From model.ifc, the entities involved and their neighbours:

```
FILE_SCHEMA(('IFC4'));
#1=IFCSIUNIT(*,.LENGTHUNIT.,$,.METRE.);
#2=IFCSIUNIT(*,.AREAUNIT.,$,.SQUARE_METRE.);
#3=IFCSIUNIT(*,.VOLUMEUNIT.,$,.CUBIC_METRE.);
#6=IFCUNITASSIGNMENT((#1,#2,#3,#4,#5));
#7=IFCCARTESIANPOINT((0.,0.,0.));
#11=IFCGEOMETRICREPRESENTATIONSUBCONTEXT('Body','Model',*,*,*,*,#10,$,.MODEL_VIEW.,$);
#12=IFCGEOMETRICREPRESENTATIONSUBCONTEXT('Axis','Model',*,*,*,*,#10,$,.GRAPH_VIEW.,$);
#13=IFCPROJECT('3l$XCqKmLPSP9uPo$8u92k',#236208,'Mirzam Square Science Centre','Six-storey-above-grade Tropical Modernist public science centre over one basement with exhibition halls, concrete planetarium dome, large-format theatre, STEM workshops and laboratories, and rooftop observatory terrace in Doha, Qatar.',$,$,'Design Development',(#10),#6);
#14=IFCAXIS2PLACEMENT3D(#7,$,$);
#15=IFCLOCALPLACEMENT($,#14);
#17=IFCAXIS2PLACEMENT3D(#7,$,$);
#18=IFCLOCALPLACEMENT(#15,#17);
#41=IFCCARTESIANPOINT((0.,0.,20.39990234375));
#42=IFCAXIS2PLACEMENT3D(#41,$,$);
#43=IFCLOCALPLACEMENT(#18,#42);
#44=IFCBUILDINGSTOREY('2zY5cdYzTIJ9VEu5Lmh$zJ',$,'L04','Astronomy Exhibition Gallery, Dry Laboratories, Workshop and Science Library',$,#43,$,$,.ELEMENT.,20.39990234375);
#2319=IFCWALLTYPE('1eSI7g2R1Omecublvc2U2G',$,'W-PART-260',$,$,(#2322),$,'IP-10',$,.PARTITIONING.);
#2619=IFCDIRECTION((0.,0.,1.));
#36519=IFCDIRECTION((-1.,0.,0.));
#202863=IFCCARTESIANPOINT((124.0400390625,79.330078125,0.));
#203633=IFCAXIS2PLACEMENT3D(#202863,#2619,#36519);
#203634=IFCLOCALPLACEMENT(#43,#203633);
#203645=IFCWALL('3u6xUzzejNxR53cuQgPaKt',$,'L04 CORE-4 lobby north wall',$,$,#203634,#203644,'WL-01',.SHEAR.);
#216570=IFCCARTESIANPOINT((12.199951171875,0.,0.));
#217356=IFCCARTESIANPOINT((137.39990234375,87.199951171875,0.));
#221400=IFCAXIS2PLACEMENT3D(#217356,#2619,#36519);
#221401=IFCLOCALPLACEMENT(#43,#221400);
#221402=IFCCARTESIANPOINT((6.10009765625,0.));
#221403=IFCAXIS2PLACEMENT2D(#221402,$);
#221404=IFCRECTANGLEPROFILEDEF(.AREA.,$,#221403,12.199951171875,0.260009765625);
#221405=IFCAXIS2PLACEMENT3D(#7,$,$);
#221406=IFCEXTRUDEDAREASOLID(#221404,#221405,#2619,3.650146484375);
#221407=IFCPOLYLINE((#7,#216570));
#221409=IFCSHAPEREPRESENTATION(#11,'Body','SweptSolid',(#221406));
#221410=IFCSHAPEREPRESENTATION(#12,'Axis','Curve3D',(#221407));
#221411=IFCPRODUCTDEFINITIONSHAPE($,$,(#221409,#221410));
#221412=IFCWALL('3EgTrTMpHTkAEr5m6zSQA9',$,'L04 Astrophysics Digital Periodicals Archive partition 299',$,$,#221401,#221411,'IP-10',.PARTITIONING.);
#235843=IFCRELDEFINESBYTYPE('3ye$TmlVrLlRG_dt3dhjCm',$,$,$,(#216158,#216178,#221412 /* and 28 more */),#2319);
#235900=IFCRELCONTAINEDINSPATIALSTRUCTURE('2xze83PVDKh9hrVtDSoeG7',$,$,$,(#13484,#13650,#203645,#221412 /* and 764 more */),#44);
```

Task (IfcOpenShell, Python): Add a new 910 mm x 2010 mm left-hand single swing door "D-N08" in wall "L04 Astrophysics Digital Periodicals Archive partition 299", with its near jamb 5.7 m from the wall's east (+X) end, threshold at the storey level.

```python
import numpy as np
import ifcopenshell
import ifcopenshell.api.feature
import ifcopenshell.api.geometry
import ifcopenshell.api.root
import ifcopenshell.api.spatial
import ifcopenshell.geom
import ifcopenshell.util.element
import ifcopenshell.util.placement
import ifcopenshell.util.representation
import ifcopenshell.util.shape
import ifcopenshell.util.unit

model = ifcopenshell.open("model.ifc")
unit_scale = ifcopenshell.util.unit.calculate_unit_scale(model)
settings = ifcopenshell.geom.settings()


def volume(element):
    """Net volume in cubic metres, openings subtracted."""
    shape = ifcopenshell.geom.create_shape(settings, element)
    return ifcopenshell.util.shape.get_volume(shape.geometry)


wall = model.by_guid("3EgTrTMpHTkAEr5m6zSQA9")
storey = ifcopenshell.util.element.get_container(wall, ifc_class="IfcBuildingStorey")
context = ifcopenshell.util.representation.get_context(model, "Model", "Body", "MODEL_VIEW")
before = volume(wall)

width, height, from_end, sill = 0.91, 2.01, 5.7, 0.0  # metres

# The wall runs along its own X axis, and the end named is its -X end.
wall_shape = ifcopenshell.geom.create_shape(settings, wall)
x, y, z = ifcopenshell.util.shape.get_vertices(wall_shape.geometry).T
start = x.min() + from_end
face, thickness = float(y.min()), float(y.max() - y.min())
wall_matrix = ifcopenshell.util.placement.get_local_placement(wall.ObjectPlacement)
level = ifcopenshell.util.placement.get_local_placement(storey.ObjectPlacement)[2, 3]


def in_wall(x, y):
    """Placement at x, y metres in the wall's axes, at sill height."""
    matrix = wall_matrix.copy()
    matrix[:, 3] = wall_matrix @ np.array([x / unit_scale, y / unit_scale, 0.0, 1.0])
    matrix[2, 3] = level + sill / unit_scale
    return matrix


# Opening: a box that overshoots both wall faces by 50 mm.
opening = ifcopenshell.api.root.create_entity(model, ifc_class="IfcOpeningElement", predefined_type="OPENING")
box = ifcopenshell.api.geometry.add_wall_representation(
    model, context=context, length=width, height=height, thickness=thickness + 0.1
)
ifcopenshell.api.geometry.assign_representation(model, product=opening, representation=box)
ifcopenshell.api.geometry.edit_object_placement(model, product=opening, matrix=in_wall(start, face - 0.05), is_si=False)
ifcopenshell.api.feature.add_feature(model, feature=opening, element=wall)

door = ifcopenshell.api.root.create_entity(model, ifc_class="IfcDoor", name="D-N08", predefined_type="DOOR")
door.OverallWidth, door.OverallHeight = width / unit_scale, height / unit_scale
door.OperationType = "SINGLE_SWING_LEFT"
body = ifcopenshell.api.geometry.add_door_representation(
    model,
    context=context,
    overall_width=door.OverallWidth,
    overall_height=door.OverallHeight,
    operation_type="SINGLE_SWING_LEFT",
    lining_properties={"LiningDepth": thickness / unit_scale, "ThresholdDepth": thickness / unit_scale},
)
ifcopenshell.api.geometry.assign_representation(model, product=door, representation=body)
ifcopenshell.api.spatial.assign_container(model, products=[door], relating_structure=storey)
ifcopenshell.api.feature.add_filling(model, opening=opening, element=door)

# The lining spans the wall, so the door starts at the wall face.
ifcopenshell.api.geometry.edit_object_placement(model, product=door, matrix=in_wall(start, face), is_si=False)

after = volume(wall)

print(f"wall volume {before:.3f} -> {after:.3f} m3")

model.write("model_updated.ifc")
```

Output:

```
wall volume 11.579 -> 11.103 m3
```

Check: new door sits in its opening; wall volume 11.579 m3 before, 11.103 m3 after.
